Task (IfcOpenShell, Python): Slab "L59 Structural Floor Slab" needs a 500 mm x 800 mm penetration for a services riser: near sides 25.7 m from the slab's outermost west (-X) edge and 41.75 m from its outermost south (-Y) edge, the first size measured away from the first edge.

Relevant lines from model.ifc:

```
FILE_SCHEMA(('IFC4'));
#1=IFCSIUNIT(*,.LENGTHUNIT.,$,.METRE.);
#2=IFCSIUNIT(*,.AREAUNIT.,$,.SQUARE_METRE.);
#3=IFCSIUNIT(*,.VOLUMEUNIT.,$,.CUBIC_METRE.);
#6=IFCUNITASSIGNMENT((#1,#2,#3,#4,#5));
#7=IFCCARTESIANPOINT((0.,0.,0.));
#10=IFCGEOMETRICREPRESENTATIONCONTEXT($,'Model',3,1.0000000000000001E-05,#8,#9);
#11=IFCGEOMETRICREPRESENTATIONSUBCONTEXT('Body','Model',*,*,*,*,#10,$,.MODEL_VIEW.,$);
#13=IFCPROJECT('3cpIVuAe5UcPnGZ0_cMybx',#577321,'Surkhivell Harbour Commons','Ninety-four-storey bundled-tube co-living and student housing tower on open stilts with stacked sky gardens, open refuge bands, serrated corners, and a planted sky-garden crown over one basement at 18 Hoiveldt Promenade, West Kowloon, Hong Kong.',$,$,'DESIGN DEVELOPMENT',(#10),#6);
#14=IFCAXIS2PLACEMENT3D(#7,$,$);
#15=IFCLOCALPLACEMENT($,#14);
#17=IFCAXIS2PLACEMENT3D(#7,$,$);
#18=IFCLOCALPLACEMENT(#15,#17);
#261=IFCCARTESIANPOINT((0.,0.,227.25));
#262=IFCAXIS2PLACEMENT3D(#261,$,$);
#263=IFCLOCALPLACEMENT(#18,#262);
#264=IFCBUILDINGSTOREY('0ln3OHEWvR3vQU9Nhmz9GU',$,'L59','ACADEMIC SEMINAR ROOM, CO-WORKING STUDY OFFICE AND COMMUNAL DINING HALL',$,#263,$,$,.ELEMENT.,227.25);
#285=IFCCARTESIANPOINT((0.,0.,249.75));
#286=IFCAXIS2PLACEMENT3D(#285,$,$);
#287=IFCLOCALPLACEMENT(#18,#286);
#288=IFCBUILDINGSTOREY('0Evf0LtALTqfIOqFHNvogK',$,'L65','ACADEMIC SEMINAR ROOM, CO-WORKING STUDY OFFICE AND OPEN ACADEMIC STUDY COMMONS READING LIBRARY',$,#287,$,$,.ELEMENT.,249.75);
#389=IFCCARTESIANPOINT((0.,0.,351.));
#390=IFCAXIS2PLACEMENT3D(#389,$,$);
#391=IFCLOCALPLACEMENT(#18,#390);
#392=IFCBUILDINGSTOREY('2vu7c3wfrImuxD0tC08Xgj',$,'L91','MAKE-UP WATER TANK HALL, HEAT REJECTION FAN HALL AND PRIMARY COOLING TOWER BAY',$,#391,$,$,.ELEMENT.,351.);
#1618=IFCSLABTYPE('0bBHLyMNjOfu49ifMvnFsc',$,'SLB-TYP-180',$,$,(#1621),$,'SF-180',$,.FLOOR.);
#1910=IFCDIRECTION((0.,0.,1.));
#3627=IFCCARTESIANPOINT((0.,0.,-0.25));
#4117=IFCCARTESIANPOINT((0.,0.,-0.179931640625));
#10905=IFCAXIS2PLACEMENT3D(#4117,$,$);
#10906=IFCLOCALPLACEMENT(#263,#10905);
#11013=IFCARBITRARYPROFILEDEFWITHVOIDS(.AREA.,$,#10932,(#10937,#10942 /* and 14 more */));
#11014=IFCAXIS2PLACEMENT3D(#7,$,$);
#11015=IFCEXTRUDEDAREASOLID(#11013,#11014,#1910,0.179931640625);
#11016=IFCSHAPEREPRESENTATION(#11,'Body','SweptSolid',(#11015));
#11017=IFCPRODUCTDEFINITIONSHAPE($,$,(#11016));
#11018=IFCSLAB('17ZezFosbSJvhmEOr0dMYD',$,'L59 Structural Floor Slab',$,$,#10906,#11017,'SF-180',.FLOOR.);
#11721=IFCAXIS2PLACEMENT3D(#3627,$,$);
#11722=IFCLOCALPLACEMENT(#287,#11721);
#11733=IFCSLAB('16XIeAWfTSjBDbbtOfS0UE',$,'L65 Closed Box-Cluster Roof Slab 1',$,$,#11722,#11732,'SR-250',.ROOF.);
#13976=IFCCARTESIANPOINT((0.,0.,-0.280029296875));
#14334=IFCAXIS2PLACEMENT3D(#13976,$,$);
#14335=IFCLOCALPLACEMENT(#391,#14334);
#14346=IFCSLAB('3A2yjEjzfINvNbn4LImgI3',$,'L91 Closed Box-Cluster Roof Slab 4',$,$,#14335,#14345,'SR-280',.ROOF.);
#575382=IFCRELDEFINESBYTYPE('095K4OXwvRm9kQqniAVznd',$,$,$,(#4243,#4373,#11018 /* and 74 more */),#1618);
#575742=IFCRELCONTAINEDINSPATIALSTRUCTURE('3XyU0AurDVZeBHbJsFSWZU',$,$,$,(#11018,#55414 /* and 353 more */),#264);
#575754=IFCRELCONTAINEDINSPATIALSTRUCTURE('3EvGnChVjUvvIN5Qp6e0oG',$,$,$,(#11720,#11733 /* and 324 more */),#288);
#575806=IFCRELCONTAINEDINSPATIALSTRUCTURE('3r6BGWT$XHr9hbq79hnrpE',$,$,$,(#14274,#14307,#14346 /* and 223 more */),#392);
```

```python
import numpy as np
import ifcopenshell
import ifcopenshell.api.feature
import ifcopenshell.api.geometry
import ifcopenshell.api.root
import ifcopenshell.geom
import ifcopenshell.util.placement
import ifcopenshell.util.representation
import ifcopenshell.util.shape
import ifcopenshell.util.unit

model = ifcopenshell.open("model.ifc")
unit_scale = ifcopenshell.util.unit.calculate_unit_scale(model)
settings = ifcopenshell.geom.settings()


def volume(element):
    """Net volume in cubic metres, openings subtracted."""
    shape = ifcopenshell.geom.create_shape(settings, element)
    return ifcopenshell.util.shape.get_volume(shape.geometry)


slab = model.by_id(11018)
before = volume(slab)

# Extent in the slab's own axes, in metres. The edges named are its -X and -Y sides.
slab_shape = ifcopenshell.geom.create_shape(settings, slab)
vertices = ifcopenshell.util.shape.get_vertices(slab_shape.geometry)
x_min, y_min, bottom = vertices.min(axis=0)
top = vertices[:, 2].max()

opening = ifcopenshell.api.root.create_entity(model, ifc_class="IfcOpeningElement", name="Services riser opening", predefined_type="OPENING")
context = ifcopenshell.util.representation.get_context(model, "Model", "Body", "MODEL_VIEW")
width, depth = 0.5, 0.8
outline = [(0.0, 0.0), (width, 0.0), (width, depth), (0.0, depth), (0.0, 0.0)]
# Overshoot both faces by 50 mm so the cut is clean.
shape = ifcopenshell.api.geometry.add_slab_representation(
    model, context=context, depth=top - bottom + 0.1, polyline=outline
)
ifcopenshell.api.geometry.assign_representation(model, product=opening, representation=shape)

matrix = ifcopenshell.util.placement.get_local_placement(slab.ObjectPlacement)
matrix[:, 3] = matrix @ np.append(np.array([x_min + 25.7, y_min + 41.75, bottom - 0.05]) / unit_scale, 1.0)
ifcopenshell.api.geometry.edit_object_placement(model, product=opening, matrix=matrix, is_si=False)
ifcopenshell.api.feature.add_feature(model, feature=opening, element=slab)

after = volume(slab)

print(f"slab volume {before:.3f} -> {after:.3f} m3")

model.write("model-out.ifc")
```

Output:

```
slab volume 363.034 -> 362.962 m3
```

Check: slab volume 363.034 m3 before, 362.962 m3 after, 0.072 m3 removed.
